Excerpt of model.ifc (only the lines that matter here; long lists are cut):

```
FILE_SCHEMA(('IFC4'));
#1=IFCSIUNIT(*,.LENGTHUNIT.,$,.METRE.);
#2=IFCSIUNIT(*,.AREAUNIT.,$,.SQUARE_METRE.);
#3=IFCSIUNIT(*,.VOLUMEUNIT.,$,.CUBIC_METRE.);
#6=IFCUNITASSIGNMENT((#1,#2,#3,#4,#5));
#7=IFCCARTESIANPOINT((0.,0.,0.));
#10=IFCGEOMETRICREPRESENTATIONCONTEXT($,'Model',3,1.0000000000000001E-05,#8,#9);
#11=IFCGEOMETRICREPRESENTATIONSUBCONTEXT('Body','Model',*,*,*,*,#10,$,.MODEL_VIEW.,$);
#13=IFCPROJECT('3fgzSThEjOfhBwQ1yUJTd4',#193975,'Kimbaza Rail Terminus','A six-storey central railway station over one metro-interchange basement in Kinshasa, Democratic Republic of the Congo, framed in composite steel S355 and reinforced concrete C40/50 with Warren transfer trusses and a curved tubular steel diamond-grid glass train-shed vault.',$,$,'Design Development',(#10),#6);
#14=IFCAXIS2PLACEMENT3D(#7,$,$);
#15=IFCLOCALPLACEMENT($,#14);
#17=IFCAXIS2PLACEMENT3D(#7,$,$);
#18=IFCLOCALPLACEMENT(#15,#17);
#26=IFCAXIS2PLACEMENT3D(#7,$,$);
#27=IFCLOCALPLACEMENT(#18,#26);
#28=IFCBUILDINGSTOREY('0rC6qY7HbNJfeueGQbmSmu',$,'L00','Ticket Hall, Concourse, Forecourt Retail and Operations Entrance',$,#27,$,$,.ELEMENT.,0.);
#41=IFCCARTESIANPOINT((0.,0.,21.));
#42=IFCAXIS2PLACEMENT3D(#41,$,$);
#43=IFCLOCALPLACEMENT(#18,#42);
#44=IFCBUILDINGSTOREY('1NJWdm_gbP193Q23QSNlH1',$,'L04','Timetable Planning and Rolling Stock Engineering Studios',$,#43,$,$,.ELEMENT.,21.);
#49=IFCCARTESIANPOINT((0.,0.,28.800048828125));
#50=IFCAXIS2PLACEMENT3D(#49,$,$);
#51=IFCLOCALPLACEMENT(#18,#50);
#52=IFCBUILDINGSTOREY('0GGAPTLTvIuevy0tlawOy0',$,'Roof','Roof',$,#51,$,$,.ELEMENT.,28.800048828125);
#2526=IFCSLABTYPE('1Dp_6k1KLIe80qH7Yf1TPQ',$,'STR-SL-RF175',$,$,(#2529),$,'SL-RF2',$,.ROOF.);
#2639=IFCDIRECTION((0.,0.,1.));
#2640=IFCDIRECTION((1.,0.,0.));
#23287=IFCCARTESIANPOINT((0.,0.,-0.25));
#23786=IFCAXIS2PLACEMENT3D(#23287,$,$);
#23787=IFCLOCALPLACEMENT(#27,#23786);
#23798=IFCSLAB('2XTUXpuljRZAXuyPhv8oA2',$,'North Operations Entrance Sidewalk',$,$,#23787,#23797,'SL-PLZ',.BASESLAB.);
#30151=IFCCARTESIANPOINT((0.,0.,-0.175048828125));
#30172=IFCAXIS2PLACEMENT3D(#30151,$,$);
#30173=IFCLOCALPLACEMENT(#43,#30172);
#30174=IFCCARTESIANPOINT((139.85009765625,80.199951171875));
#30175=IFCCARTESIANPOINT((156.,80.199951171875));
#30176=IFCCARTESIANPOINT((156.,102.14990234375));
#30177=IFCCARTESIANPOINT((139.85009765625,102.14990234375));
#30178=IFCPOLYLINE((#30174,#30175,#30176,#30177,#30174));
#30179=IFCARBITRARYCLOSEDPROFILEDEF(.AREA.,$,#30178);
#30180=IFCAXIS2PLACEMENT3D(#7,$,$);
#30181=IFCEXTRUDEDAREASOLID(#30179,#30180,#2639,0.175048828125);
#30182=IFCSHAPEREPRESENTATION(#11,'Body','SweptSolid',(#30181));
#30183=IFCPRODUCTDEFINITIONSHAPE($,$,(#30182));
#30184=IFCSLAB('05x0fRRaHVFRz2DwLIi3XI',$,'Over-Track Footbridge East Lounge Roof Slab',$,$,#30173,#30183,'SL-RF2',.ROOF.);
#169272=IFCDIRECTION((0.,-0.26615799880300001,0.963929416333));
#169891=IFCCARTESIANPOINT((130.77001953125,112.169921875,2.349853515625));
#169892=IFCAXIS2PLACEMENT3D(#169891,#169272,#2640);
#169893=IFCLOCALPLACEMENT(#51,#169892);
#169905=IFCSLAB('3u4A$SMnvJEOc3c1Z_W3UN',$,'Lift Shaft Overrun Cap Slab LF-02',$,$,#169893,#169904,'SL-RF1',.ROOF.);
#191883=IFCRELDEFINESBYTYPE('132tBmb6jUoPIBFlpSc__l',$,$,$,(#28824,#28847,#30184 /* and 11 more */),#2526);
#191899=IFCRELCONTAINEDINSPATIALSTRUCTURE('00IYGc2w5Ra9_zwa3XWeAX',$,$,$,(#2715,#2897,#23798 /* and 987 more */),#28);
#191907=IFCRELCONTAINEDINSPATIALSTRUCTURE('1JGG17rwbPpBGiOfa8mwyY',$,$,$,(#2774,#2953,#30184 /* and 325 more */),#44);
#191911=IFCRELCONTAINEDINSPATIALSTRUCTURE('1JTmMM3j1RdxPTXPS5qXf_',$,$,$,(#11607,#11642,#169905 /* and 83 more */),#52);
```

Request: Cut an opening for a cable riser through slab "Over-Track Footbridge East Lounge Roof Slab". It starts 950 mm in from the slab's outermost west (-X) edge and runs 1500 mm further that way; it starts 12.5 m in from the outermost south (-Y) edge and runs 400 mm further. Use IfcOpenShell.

```python
import numpy as np
import ifcopenshell
import ifcopenshell.api.feature
import ifcopenshell.api.geometry
import ifcopenshell.api.root
import ifcopenshell.geom
import ifcopenshell.util.placement
import ifcopenshell.util.representation
import ifcopenshell.util.shape
import ifcopenshell.util.unit

model = ifcopenshell.open("model.ifc")
unit_scale = ifcopenshell.util.unit.calculate_unit_scale(model)
settings = ifcopenshell.geom.settings()


def volume(element):
    """Net volume in cubic metres, openings subtracted."""
    shape = ifcopenshell.geom.create_shape(settings, element)
    return ifcopenshell.util.shape.get_volume(shape.geometry)


slab = model.by_guid("05x0fRRaHVFRz2DwLIi3XI")
before = volume(slab)

# Extent in the slab's own axes, in metres. The edges named are its -X and -Y sides.
slab_shape = ifcopenshell.geom.create_shape(settings, slab)
vertices = ifcopenshell.util.shape.get_vertices(slab_shape.geometry)
x_min, y_min, bottom = vertices.min(axis=0)
top = vertices[:, 2].max()

opening = ifcopenshell.api.root.create_entity(model, ifc_class="IfcOpeningElement", name="Cable riser opening", predefined_type="OPENING")
context = ifcopenshell.util.representation.get_context(model, "Model", "Body", "MODEL_VIEW")
width, depth = 1.5, 0.4
outline = [(0.0, 0.0), (width, 0.0), (width, depth), (0.0, depth), (0.0, 0.0)]
# Overshoot both faces by 50 mm so the cut is clean.
shape = ifcopenshell.api.geometry.add_slab_representation(
    model, context=context, depth=top - bottom + 0.1, polyline=outline
)
ifcopenshell.api.geometry.assign_representation(model, product=opening, representation=shape)

matrix = ifcopenshell.util.placement.get_local_placement(slab.ObjectPlacement)
matrix[:, 3] = matrix @ np.append(np.array([x_min + 0.95, y_min + 12.5, bottom - 0.05]) / unit_scale, 1.0)
ifcopenshell.api.geometry.edit_object_placement(model, product=opening, matrix=matrix, is_si=False)
ifcopenshell.api.feature.add_feature(model, feature=opening, element=slab)

after = volume(slab)

print(f"slab volume {before:.3f} -> {after:.3f} m3")

model.write("model_edited.ifc")
```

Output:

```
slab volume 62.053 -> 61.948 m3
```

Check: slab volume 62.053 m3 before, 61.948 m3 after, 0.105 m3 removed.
